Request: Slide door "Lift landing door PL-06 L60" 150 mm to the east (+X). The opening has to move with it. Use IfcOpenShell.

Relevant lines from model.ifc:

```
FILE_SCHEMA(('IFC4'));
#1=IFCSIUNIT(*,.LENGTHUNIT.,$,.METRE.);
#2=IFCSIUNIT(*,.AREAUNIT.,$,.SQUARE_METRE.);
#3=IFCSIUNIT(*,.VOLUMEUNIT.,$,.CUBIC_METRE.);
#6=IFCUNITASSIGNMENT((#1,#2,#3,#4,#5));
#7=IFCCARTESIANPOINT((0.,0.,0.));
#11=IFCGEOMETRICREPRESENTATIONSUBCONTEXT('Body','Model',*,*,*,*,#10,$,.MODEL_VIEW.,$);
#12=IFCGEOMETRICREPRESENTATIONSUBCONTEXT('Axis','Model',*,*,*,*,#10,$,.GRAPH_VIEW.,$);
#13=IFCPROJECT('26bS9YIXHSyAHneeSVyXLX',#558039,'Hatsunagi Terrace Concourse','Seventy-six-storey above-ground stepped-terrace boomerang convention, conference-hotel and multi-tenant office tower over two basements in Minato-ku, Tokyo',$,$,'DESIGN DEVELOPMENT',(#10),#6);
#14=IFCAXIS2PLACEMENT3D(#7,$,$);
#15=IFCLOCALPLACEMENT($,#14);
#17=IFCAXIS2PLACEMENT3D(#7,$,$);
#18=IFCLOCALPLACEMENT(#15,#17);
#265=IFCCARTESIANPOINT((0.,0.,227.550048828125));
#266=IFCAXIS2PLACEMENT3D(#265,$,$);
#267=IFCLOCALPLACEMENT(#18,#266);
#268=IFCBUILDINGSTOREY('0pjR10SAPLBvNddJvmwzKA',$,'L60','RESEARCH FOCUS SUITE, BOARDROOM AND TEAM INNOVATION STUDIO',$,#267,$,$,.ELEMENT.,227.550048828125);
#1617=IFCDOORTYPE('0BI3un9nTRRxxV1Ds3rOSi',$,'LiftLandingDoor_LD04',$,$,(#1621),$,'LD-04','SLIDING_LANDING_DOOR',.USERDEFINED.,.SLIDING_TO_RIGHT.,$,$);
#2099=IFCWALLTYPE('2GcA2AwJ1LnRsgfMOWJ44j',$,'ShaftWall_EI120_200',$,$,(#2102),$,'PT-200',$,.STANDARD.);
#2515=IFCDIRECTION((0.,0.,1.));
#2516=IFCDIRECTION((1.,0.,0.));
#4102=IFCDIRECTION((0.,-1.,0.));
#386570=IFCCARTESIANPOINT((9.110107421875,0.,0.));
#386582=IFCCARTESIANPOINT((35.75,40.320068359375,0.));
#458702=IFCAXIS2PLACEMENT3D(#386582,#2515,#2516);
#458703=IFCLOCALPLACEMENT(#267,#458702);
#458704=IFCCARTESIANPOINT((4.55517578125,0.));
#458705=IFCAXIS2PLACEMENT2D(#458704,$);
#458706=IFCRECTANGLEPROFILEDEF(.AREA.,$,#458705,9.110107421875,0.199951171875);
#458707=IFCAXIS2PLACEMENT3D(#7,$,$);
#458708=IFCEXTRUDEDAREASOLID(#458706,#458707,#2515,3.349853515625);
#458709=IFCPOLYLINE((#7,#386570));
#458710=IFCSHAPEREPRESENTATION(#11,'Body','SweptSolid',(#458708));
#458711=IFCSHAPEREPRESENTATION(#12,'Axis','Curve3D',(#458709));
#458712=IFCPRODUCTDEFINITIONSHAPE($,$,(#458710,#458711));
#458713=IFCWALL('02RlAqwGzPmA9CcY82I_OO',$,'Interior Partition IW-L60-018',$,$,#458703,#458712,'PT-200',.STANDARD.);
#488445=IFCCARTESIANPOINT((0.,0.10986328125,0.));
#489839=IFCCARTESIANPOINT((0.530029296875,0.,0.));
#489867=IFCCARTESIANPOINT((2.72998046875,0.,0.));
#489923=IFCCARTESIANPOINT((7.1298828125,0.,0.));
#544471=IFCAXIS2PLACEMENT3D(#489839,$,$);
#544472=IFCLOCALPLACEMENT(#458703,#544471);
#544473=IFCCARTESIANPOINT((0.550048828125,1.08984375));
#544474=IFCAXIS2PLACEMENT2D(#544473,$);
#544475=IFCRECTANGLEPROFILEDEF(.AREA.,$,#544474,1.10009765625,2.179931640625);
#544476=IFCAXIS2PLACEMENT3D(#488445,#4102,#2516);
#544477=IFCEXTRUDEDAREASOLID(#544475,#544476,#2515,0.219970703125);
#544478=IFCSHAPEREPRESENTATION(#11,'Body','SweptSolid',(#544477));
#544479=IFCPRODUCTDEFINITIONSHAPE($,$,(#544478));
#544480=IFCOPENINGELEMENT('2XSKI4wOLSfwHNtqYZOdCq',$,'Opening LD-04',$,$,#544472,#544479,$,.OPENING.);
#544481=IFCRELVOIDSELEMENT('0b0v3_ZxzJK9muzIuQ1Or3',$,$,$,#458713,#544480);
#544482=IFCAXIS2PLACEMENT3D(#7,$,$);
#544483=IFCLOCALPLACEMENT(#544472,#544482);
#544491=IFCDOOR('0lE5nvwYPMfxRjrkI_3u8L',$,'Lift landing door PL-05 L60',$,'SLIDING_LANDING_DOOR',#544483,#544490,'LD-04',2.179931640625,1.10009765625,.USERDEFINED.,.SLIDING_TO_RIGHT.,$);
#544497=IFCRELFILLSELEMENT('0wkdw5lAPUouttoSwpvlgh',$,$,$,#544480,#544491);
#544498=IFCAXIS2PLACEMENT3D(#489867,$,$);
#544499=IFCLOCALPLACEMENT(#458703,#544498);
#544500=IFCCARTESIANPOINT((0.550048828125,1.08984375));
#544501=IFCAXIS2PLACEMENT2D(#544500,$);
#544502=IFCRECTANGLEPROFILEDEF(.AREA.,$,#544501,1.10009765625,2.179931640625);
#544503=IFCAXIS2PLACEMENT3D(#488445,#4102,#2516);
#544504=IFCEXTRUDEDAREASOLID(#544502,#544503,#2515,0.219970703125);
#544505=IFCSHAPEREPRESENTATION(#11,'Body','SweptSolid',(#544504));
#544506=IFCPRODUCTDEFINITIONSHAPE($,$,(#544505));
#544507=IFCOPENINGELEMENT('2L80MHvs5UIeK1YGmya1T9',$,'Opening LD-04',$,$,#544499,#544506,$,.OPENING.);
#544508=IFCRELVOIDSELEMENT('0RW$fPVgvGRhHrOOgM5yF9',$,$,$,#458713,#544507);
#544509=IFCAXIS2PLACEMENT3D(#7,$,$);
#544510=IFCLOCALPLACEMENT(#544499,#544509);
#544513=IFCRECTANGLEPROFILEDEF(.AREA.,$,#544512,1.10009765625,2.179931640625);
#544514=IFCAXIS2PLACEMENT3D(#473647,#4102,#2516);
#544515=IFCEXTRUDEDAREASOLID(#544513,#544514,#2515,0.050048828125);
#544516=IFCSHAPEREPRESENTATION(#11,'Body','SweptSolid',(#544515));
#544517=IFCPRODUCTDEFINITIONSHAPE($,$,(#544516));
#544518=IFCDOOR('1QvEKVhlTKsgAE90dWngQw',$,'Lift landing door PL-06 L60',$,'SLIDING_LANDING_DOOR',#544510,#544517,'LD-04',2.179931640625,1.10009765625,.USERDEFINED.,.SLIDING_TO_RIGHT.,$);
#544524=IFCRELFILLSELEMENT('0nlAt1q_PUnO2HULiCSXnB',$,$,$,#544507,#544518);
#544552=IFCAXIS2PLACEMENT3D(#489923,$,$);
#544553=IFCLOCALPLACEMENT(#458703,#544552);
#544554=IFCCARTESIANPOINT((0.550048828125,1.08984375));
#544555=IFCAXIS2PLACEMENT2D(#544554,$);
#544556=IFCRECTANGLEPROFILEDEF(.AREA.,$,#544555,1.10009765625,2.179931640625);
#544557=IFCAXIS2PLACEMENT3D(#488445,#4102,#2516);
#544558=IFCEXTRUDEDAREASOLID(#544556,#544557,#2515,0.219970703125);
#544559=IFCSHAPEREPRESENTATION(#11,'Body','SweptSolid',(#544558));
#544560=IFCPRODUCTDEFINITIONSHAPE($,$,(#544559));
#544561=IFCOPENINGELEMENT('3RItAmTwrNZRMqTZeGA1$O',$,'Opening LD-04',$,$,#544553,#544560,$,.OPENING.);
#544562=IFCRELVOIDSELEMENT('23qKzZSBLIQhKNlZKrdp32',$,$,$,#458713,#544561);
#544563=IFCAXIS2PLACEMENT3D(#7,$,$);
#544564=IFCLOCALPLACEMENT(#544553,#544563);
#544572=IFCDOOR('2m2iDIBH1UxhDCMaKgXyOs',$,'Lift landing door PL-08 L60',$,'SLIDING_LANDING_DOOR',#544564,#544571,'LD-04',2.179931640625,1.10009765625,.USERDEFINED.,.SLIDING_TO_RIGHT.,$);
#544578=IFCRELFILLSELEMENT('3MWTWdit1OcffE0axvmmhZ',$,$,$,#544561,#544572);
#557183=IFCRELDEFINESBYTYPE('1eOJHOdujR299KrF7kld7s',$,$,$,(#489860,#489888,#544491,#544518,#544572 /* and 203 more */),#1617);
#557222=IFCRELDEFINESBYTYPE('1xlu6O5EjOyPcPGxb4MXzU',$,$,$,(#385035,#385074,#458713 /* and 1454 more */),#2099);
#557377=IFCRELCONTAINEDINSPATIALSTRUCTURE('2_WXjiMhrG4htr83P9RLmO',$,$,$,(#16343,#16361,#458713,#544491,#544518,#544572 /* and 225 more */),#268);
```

```python
import ifcopenshell
import ifcopenshell.api.geometry
import ifcopenshell.util.placement
import ifcopenshell.util.unit

model = ifcopenshell.open("model.ifc")
unit_scale = ifcopenshell.util.unit.calculate_unit_scale(model)

door = model.by_guid("1QvEKVhlTKsgAE90dWngQw")
opening = door.FillsVoids[0].RelatingOpeningElement
wall = opening.VoidsElements[0].RelatingBuildingElement

wall_matrix = ifcopenshell.util.placement.get_local_placement(wall.ObjectPlacement)
shift = wall_matrix[:3, 0] * 0.15 / unit_scale
before = ifcopenshell.util.placement.get_local_placement(door.ObjectPlacement)[:3, 3].copy()

# The door is placed relative to its opening, so it follows when the opening moves.
matrix = ifcopenshell.util.placement.get_local_placement(opening.ObjectPlacement)
matrix[:3, 3] += shift
ifcopenshell.api.geometry.edit_object_placement(
    model, product=opening, matrix=matrix, is_si=False, should_transform_children=True
)

after = ifcopenshell.util.placement.get_local_placement(door.ObjectPlacement)[:3, 3]
print("door moved by", (after - before).round(3) + 0.0)

model.write("model_updated.ifc")
```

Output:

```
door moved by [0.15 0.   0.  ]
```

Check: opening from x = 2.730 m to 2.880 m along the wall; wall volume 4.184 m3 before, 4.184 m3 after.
